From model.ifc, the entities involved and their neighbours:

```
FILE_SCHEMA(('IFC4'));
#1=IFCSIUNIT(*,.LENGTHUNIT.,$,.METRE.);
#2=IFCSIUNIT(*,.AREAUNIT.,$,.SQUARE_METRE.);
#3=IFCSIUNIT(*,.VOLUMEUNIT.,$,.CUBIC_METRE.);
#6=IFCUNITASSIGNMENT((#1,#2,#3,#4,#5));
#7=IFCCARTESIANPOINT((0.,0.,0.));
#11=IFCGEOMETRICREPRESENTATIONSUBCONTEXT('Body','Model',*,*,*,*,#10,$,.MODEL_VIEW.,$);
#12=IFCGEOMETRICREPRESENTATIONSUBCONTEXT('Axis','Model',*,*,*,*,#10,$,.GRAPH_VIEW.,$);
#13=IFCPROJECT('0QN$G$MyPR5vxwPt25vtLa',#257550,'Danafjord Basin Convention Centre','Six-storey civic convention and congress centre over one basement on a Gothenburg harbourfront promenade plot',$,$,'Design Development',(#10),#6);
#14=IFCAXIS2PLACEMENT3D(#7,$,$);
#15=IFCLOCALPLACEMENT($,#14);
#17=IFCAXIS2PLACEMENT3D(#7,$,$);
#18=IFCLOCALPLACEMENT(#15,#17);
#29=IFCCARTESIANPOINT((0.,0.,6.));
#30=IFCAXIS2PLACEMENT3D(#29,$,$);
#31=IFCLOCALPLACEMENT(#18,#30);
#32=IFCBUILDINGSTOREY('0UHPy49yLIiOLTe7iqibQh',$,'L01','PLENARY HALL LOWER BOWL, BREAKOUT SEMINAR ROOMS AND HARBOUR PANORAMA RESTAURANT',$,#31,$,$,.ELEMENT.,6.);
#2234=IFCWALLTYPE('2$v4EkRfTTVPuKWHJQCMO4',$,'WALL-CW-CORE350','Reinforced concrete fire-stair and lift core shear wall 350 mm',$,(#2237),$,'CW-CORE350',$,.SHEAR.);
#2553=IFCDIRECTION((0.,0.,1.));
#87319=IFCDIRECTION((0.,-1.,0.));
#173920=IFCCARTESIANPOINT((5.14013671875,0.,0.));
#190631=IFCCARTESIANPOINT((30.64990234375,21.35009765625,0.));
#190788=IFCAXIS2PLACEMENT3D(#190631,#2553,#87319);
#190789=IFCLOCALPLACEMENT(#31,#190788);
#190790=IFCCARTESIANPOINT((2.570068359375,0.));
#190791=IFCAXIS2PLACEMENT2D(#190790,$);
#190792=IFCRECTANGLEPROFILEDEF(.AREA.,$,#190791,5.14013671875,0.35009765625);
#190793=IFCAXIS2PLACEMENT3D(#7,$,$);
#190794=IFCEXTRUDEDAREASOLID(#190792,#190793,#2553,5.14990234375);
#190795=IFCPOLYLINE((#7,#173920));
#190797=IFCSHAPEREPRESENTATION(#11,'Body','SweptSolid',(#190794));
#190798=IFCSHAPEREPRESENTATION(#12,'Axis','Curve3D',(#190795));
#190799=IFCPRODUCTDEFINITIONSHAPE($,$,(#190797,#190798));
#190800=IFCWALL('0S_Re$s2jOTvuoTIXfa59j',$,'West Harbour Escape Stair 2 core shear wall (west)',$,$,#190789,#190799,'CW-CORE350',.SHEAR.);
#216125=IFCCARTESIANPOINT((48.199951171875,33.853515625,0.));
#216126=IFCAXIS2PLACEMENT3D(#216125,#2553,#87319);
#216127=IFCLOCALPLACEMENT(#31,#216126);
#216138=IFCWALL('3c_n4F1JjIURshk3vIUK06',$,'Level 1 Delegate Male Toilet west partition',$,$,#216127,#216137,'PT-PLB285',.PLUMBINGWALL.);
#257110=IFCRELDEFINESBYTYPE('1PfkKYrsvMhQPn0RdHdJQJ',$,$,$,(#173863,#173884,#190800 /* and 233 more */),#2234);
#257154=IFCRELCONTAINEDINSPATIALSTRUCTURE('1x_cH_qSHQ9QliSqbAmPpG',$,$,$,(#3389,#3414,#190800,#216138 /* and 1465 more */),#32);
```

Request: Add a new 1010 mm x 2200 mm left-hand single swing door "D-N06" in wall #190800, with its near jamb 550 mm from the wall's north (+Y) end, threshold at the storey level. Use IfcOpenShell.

```python
import numpy as np
import ifcopenshell
import ifcopenshell.api.feature
import ifcopenshell.api.geometry
import ifcopenshell.api.root
import ifcopenshell.api.spatial
import ifcopenshell.geom
import ifcopenshell.util.element
import ifcopenshell.util.placement
import ifcopenshell.util.representation
import ifcopenshell.util.shape
import ifcopenshell.util.unit

model = ifcopenshell.open("model.ifc")
unit_scale = ifcopenshell.util.unit.calculate_unit_scale(model)
settings = ifcopenshell.geom.settings()


def volume(element):
    """Net volume in cubic metres, openings subtracted."""
    shape = ifcopenshell.geom.create_shape(settings, element)
    return ifcopenshell.util.shape.get_volume(shape.geometry)


wall = model.by_id(190800)
storey = ifcopenshell.util.element.get_container(wall, ifc_class="IfcBuildingStorey")
context = ifcopenshell.util.representation.get_context(model, "Model", "Body", "MODEL_VIEW")
before = volume(wall)

width, height, from_end, sill = 1.01, 2.2, 0.55, 0.0  # metres

# The wall runs along its own X axis, and the end named is its -X end.
wall_shape = ifcopenshell.geom.create_shape(settings, wall)
x, y, z = ifcopenshell.util.shape.get_vertices(wall_shape.geometry).T
start = x.min() + from_end
face, thickness = float(y.min()), float(y.max() - y.min())
wall_matrix = ifcopenshell.util.placement.get_local_placement(wall.ObjectPlacement)
level = ifcopenshell.util.placement.get_local_placement(storey.ObjectPlacement)[2, 3]


def in_wall(x, y):
    """Placement at x, y metres in the wall's axes, at sill height."""
    matrix = wall_matrix.copy()
    matrix[:, 3] = wall_matrix @ np.array([x / unit_scale, y / unit_scale, 0.0, 1.0])
    matrix[2, 3] = level + sill / unit_scale
    return matrix


# Opening: a box that overshoots both wall faces by 50 mm.
opening = ifcopenshell.api.root.create_entity(model, ifc_class="IfcOpeningElement", predefined_type="OPENING")
box = ifcopenshell.api.geometry.add_wall_representation(
    model, context=context, length=width, height=height, thickness=thickness + 0.1
)
ifcopenshell.api.geometry.assign_representation(model, product=opening, representation=box)
ifcopenshell.api.geometry.edit_object_placement(model, product=opening, matrix=in_wall(start, face - 0.05), is_si=False)
ifcopenshell.api.feature.add_feature(model, feature=opening, element=wall)

door = ifcopenshell.api.root.create_entity(model, ifc_class="IfcDoor", name="D-N06", predefined_type="DOOR")
door.OverallWidth, door.OverallHeight = width / unit_scale, height / unit_scale
door.OperationType = "SINGLE_SWING_LEFT"
body = ifcopenshell.api.geometry.add_door_representation(
    model,
    context=context,
    overall_width=door.OverallWidth,
    overall_height=door.OverallHeight,
    operation_type="SINGLE_SWING_LEFT",
    lining_properties={"LiningDepth": thickness / unit_scale, "ThresholdDepth": thickness / unit_scale},
)
ifcopenshell.api.geometry.assign_representation(model, product=door, representation=body)
ifcopenshell.api.spatial.assign_container(model, products=[door], relating_structure=storey)
ifcopenshell.api.feature.add_filling(model, opening=opening, element=door)

# The lining spans the wall, so the door starts at the wall face.
ifcopenshell.api.geometry.edit_object_placement(model, product=door, matrix=in_wall(start, face), is_si=False)

after = volume(wall)

print(f"wall volume {before:.3f} -> {after:.3f} m3")

model.write("model_v2.ifc")
```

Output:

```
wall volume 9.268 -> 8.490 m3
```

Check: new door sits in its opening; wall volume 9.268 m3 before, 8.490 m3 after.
